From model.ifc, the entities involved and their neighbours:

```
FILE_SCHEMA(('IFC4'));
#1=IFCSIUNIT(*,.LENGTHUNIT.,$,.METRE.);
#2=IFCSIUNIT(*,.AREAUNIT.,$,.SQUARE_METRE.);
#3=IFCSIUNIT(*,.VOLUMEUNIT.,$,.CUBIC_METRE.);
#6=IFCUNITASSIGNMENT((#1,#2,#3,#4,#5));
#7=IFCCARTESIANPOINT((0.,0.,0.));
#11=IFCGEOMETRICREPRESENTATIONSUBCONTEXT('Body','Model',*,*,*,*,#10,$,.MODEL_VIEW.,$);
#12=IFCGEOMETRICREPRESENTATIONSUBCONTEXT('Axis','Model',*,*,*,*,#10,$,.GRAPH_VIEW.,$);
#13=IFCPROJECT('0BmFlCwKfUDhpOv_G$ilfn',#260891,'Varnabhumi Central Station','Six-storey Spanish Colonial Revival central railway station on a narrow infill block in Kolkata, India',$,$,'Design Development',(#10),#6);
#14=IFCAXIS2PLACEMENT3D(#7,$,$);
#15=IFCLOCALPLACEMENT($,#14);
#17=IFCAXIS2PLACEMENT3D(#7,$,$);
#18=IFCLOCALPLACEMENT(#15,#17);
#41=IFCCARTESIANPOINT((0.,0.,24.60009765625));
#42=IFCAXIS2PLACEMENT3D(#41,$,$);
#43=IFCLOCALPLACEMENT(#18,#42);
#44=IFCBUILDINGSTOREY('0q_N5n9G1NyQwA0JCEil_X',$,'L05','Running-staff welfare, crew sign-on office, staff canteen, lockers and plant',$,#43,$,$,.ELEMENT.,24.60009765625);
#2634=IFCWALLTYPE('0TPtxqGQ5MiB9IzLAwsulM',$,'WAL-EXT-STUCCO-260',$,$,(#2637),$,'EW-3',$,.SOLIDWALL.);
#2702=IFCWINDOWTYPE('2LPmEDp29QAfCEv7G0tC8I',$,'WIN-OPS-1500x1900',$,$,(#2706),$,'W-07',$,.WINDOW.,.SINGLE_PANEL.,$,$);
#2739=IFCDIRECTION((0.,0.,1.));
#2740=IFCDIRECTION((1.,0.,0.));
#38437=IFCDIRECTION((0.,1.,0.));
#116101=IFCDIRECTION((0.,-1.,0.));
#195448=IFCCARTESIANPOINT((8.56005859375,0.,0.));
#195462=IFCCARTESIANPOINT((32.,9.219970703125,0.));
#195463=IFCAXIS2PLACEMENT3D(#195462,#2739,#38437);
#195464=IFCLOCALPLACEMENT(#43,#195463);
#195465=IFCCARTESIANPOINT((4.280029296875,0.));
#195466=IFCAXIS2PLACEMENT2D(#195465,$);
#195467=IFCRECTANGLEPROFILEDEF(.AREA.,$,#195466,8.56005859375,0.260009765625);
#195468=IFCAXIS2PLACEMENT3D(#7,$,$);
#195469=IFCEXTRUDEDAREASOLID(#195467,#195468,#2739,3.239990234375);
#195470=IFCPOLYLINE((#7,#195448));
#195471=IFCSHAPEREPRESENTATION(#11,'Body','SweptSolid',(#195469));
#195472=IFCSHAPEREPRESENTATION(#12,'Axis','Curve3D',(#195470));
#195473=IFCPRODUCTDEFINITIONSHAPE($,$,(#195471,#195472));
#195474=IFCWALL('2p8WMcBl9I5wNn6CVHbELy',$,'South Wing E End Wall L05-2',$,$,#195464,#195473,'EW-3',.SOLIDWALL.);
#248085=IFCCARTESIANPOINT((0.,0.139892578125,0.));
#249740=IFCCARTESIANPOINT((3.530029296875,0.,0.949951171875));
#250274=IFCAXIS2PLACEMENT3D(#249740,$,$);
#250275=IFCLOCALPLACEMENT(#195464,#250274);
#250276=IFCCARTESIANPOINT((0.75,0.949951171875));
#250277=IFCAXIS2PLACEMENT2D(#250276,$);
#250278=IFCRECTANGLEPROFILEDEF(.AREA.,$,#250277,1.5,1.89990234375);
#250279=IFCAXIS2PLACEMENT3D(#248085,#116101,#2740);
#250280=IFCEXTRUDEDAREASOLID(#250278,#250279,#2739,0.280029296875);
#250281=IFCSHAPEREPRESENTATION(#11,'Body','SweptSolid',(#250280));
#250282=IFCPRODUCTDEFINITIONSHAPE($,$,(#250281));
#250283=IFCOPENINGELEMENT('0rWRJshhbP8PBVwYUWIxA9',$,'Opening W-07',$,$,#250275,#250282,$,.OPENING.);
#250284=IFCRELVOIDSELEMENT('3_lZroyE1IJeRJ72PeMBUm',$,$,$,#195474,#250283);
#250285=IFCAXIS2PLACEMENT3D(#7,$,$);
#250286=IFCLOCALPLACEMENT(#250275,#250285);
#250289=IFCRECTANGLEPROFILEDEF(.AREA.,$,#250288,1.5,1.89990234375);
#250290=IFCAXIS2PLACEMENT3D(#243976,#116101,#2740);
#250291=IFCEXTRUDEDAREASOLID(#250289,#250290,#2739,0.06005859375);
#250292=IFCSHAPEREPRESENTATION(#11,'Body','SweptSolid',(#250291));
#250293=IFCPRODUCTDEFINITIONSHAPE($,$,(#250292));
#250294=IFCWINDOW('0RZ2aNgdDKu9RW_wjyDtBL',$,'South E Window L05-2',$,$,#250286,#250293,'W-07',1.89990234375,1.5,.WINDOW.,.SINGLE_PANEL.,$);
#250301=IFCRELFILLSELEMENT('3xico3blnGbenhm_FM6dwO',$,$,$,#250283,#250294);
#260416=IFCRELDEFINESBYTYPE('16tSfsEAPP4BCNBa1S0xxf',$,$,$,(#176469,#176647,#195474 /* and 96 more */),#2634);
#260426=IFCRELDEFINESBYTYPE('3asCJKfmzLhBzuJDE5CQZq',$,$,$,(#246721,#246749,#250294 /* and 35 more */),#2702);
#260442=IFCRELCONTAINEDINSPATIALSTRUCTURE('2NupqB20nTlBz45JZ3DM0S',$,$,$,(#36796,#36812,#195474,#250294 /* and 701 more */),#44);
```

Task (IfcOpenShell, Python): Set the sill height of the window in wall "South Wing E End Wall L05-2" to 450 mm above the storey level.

```python
import numpy as np
import ifcopenshell
import ifcopenshell.api.geometry
import ifcopenshell.geom
import ifcopenshell.util.element
import ifcopenshell.util.placement
import ifcopenshell.util.shape
import ifcopenshell.util.unit

model = ifcopenshell.open("model.ifc")
unit_scale = ifcopenshell.util.unit.calculate_unit_scale(model)

window = model.by_guid("0RZ2aNgdDKu9RW_wjyDtBL")
opening = window.FillsVoids[0].RelatingOpeningElement
storey = ifcopenshell.util.element.get_container(window, ifc_class="IfcBuildingStorey")
level = ifcopenshell.util.placement.get_local_placement(storey.ObjectPlacement)[2, 3]

# The opening's origin need not be at the sill, so measure its lowest point.
shape = ifcopenshell.geom.create_shape(ifcopenshell.geom.settings(), opening)
bottom = ifcopenshell.util.shape.get_shape_bottom_elevation(shape, shape.geometry) / unit_scale
dz = level + 0.45 / unit_scale - bottom

shift = np.array([0.0, 0.0, dz])
# The window is placed relative to its opening, so it follows when the opening moves.
matrix = ifcopenshell.util.placement.get_local_placement(opening.ObjectPlacement)
matrix[:3, 3] += shift
ifcopenshell.api.geometry.edit_object_placement(
    model, product=opening, matrix=matrix, is_si=False, should_transform_children=True
)

print(f"moved by {dz * unit_scale:+.3f} m")

model.write("model-out.ifc")
```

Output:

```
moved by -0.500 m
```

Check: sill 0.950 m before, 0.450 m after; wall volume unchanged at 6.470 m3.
